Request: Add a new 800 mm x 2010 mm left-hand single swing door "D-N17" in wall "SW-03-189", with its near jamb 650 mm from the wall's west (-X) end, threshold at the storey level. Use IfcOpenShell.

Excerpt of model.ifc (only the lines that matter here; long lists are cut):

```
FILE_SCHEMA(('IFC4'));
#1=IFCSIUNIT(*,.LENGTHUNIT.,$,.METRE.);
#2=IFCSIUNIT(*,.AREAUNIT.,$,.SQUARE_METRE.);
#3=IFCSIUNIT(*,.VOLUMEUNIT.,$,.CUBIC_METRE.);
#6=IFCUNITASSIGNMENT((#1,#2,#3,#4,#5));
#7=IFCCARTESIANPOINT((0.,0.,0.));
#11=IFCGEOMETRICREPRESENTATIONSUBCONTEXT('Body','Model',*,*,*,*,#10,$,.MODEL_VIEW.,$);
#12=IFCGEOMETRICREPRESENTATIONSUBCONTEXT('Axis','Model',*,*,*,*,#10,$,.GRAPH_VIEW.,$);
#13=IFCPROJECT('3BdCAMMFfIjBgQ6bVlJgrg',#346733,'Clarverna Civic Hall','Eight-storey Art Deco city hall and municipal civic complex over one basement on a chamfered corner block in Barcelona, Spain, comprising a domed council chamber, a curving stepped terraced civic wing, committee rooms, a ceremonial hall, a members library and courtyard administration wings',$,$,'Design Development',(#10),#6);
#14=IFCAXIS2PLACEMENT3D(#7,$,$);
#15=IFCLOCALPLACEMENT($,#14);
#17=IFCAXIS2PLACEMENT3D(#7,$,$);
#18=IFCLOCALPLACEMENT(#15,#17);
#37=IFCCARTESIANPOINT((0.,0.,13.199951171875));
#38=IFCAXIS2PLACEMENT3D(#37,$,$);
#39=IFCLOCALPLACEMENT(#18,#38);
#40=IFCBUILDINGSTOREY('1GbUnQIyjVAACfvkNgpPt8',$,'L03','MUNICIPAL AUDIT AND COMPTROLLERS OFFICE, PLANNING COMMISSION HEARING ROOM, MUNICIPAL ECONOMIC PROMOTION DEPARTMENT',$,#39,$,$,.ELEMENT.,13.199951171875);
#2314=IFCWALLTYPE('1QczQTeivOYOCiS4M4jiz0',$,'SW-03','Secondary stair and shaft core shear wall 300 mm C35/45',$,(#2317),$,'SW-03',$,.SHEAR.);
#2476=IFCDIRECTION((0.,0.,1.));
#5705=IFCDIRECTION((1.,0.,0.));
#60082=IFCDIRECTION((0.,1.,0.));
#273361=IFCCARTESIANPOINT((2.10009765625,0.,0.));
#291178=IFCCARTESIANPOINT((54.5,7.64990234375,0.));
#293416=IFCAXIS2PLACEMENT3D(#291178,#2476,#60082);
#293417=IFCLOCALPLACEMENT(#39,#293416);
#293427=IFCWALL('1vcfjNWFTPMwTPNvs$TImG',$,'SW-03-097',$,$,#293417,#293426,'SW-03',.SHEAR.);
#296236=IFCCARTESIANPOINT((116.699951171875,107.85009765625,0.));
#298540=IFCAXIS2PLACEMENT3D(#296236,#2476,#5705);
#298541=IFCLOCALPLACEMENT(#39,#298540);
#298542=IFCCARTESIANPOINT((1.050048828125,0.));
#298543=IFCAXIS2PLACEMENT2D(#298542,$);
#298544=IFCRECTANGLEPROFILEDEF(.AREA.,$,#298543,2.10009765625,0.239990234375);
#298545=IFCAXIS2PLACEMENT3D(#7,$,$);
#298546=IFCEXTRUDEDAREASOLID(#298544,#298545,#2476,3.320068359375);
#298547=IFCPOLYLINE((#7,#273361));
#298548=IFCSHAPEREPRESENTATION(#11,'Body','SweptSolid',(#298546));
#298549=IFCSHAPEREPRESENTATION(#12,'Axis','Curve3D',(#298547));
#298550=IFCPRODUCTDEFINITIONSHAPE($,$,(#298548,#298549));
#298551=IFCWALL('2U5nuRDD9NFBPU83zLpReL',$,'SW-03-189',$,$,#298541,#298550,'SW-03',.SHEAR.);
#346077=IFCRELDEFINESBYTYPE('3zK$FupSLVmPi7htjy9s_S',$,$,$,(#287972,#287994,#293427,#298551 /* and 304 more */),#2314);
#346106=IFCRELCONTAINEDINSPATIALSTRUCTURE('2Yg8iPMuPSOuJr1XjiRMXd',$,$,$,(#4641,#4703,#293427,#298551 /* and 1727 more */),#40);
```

```python
import numpy as np
import ifcopenshell
import ifcopenshell.api.feature
import ifcopenshell.api.geometry
import ifcopenshell.api.root
import ifcopenshell.api.spatial
import ifcopenshell.geom
import ifcopenshell.util.element
import ifcopenshell.util.placement
import ifcopenshell.util.representation
import ifcopenshell.util.shape
import ifcopenshell.util.unit

model = ifcopenshell.open("model.ifc")
unit_scale = ifcopenshell.util.unit.calculate_unit_scale(model)
settings = ifcopenshell.geom.settings()


def volume(element):
    """Net volume in cubic metres, openings subtracted."""
    shape = ifcopenshell.geom.create_shape(settings, element)
    return ifcopenshell.util.shape.get_volume(shape.geometry)


wall = model.by_guid("2U5nuRDD9NFBPU83zLpReL")
storey = ifcopenshell.util.element.get_container(wall, ifc_class="IfcBuildingStorey")
context = ifcopenshell.util.representation.get_context(model, "Model", "Body", "MODEL_VIEW")
before = volume(wall)

width, height, from_end, sill = 0.8, 2.01, 0.65, 0.0  # metres

# The wall runs along its own X axis, and the end named is its -X end.
wall_shape = ifcopenshell.geom.create_shape(settings, wall)
x, y, z = ifcopenshell.util.shape.get_vertices(wall_shape.geometry).T
start = x.min() + from_end
face, thickness = float(y.min()), float(y.max() - y.min())
wall_matrix = ifcopenshell.util.placement.get_local_placement(wall.ObjectPlacement)
level = ifcopenshell.util.placement.get_local_placement(storey.ObjectPlacement)[2, 3]


def in_wall(x, y):
    """Placement at x, y metres in the wall's axes, at sill height."""
    matrix = wall_matrix.copy()
    matrix[:, 3] = wall_matrix @ np.array([x / unit_scale, y / unit_scale, 0.0, 1.0])
    matrix[2, 3] = level + sill / unit_scale
    return matrix


# Opening: a box that overshoots both wall faces by 50 mm.
opening = ifcopenshell.api.root.create_entity(model, ifc_class="IfcOpeningElement", predefined_type="OPENING")
box = ifcopenshell.api.geometry.add_wall_representation(
    model, context=context, length=width, height=height, thickness=thickness + 0.1
)
ifcopenshell.api.geometry.assign_representation(model, product=opening, representation=box)
ifcopenshell.api.geometry.edit_object_placement(model, product=opening, matrix=in_wall(start, face - 0.05), is_si=False)
ifcopenshell.api.feature.add_feature(model, feature=opening, element=wall)

door = ifcopenshell.api.root.create_entity(model, ifc_class="IfcDoor", name="D-N17", predefined_type="DOOR")
door.OverallWidth, door.OverallHeight = width / unit_scale, height / unit_scale
door.OperationType = "SINGLE_SWING_LEFT"
body = ifcopenshell.api.geometry.add_door_representation(
    model,
    context=context,
    overall_width=door.OverallWidth,
    overall_height=door.OverallHeight,
    operation_type="SINGLE_SWING_LEFT",
    lining_properties={"LiningDepth": thickness / unit_scale, "ThresholdDepth": thickness / unit_scale},
)
ifcopenshell.api.geometry.assign_representation(model, product=door, representation=body)
ifcopenshell.api.spatial.assign_container(model, products=[door], relating_structure=storey)
ifcopenshell.api.feature.add_filling(model, opening=opening, element=door)

# The lining spans the wall, so the door starts at the wall face.
ifcopenshell.api.geometry.edit_object_placement(model, product=door, matrix=in_wall(start, face), is_si=False)

after = volume(wall)

print(f"wall volume {before:.3f} -> {after:.3f} m3")

model.write("model_updated.ifc")
```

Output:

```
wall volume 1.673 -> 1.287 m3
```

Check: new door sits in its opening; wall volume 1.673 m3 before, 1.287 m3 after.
